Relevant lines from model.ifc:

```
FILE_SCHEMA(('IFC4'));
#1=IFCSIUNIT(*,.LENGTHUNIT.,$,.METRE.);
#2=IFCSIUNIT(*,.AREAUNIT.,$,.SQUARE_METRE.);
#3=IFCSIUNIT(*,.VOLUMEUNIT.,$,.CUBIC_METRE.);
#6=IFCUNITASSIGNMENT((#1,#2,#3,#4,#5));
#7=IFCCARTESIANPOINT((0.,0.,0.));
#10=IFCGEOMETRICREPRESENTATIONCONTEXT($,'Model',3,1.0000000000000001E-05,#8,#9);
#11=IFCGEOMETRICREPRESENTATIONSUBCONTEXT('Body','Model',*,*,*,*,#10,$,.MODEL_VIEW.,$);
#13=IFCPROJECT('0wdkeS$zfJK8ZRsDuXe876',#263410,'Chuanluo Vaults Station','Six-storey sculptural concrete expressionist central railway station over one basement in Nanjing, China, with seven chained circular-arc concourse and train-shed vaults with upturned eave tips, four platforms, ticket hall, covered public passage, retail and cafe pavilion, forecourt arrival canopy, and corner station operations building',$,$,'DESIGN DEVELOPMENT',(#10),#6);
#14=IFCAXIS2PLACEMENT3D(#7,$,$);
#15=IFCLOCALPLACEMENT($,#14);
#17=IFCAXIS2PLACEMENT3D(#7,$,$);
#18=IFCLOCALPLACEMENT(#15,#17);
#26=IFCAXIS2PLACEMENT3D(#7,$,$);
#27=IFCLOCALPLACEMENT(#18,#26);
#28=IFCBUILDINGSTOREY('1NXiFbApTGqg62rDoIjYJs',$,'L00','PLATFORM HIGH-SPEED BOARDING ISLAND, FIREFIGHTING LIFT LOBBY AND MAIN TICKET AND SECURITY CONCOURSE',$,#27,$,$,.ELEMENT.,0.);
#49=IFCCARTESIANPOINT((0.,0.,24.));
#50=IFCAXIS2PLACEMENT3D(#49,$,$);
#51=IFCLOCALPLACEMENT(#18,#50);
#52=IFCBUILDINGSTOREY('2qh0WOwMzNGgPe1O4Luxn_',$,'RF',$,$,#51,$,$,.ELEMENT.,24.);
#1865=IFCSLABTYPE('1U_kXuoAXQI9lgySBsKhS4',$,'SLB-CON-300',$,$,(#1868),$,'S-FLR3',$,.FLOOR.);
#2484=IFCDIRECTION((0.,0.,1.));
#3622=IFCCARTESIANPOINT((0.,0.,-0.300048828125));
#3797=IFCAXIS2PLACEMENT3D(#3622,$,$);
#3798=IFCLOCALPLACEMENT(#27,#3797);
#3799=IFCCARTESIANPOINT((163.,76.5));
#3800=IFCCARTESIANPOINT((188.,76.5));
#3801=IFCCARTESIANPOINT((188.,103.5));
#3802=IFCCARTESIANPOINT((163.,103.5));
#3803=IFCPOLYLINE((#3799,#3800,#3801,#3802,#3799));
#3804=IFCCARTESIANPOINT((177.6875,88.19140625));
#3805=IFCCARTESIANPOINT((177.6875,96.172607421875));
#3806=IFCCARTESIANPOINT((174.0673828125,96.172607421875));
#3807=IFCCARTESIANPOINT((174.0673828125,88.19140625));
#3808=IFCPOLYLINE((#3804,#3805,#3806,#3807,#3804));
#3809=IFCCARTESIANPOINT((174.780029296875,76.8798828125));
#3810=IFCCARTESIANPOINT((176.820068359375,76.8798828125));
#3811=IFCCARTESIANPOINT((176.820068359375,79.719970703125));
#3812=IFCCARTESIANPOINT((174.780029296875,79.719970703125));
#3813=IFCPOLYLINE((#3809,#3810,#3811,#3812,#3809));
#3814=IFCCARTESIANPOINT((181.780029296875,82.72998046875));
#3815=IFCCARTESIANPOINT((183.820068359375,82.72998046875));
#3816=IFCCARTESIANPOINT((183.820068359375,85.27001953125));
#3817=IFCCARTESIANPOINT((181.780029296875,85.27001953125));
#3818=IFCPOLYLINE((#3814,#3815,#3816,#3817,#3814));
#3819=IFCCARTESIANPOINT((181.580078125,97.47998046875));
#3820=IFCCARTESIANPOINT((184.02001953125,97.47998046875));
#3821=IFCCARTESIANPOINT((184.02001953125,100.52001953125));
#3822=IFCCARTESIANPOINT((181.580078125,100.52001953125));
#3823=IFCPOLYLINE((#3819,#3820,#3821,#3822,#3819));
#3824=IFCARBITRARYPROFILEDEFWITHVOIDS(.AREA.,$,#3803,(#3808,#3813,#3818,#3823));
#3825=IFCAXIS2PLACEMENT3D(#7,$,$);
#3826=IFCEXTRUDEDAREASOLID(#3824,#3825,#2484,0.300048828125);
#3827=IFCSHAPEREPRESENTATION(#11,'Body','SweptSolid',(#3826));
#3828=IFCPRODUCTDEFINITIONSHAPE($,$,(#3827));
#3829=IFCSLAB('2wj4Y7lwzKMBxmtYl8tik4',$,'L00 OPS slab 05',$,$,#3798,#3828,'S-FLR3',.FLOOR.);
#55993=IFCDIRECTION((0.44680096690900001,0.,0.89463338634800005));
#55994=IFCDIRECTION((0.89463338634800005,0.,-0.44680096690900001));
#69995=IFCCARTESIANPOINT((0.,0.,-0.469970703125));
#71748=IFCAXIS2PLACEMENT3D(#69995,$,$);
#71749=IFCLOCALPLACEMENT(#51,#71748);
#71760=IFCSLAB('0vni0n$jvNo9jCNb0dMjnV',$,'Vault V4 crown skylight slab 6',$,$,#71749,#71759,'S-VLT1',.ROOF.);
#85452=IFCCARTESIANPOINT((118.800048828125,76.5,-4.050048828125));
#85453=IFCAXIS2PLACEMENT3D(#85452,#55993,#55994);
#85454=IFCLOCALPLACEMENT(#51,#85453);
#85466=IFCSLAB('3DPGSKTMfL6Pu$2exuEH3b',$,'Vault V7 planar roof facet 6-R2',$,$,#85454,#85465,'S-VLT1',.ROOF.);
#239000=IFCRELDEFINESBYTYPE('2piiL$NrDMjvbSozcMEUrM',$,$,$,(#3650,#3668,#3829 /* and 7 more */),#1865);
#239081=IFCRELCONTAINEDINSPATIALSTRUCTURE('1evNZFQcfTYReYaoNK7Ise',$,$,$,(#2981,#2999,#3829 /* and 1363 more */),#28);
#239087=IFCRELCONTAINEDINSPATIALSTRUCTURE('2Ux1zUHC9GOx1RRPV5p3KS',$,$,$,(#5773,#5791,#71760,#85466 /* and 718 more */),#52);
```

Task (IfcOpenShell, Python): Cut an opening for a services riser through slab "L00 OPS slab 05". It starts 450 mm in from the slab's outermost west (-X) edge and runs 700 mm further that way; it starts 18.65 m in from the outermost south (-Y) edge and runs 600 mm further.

```python
import numpy as np
import ifcopenshell
import ifcopenshell.api.feature
import ifcopenshell.api.geometry
import ifcopenshell.api.root
import ifcopenshell.geom
import ifcopenshell.util.placement
import ifcopenshell.util.representation
import ifcopenshell.util.shape
import ifcopenshell.util.unit

model = ifcopenshell.open("model.ifc")
unit_scale = ifcopenshell.util.unit.calculate_unit_scale(model)
settings = ifcopenshell.geom.settings()


def volume(element):
    """Net volume in cubic metres, openings subtracted."""
    shape = ifcopenshell.geom.create_shape(settings, element)
    return ifcopenshell.util.shape.get_volume(shape.geometry)


slab = model.by_id(3829)
before = volume(slab)

# Extent in the slab's own axes, in metres. The edges named are its -X and -Y sides.
slab_shape = ifcopenshell.geom.create_shape(settings, slab)
vertices = ifcopenshell.util.shape.get_vertices(slab_shape.geometry)
x_min, y_min, bottom = vertices.min(axis=0)
top = vertices[:, 2].max()

opening = ifcopenshell.api.root.create_entity(model, ifc_class="IfcOpeningElement", name="Services riser opening", predefined_type="OPENING")
context = ifcopenshell.util.representation.get_context(model, "Model", "Body", "MODEL_VIEW")
width, depth = 0.7, 0.6
outline = [(0.0, 0.0), (width, 0.0), (width, depth), (0.0, depth), (0.0, 0.0)]
# Overshoot both faces by 50 mm so the cut is clean.
shape = ifcopenshell.api.geometry.add_slab_representation(
    model, context=context, depth=top - bottom + 0.1, polyline=outline
)
ifcopenshell.api.geometry.assign_representation(model, product=opening, representation=shape)

matrix = ifcopenshell.util.placement.get_local_placement(slab.ObjectPlacement)
matrix[:, 3] = matrix @ np.append(np.array([x_min + 0.45, y_min + 18.65, bottom - 0.05]) / unit_scale, 1.0)
ifcopenshell.api.geometry.edit_object_placement(model, product=opening, matrix=matrix, is_si=False)
ifcopenshell.api.feature.add_feature(model, feature=opening, element=slab)

after = volume(slab)

print(f"slab volume {before:.3f} -> {after:.3f} m3")

model.write("model_edited.ifc")
```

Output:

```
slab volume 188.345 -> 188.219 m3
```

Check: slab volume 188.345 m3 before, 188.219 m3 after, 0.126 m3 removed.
